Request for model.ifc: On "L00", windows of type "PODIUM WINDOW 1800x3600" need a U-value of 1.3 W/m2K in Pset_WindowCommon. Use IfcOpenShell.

First a look at what the model holds.

```python
import ifcopenshell
import ifcopenshell.util.element

model = ifcopenshell.open("model.ifc")
print(model.schema)
storey = next(s for s in model.by_type("IfcBuildingStorey") if s.Name == "L00")
windows = [e for e in ifcopenshell.util.element.get_decomposition(storey) if e.is_a("IfcWindow")]
seen = {}
for e in windows:
    element_type = ifcopenshell.util.element.get_type(e)
    key = (element_type.Name if element_type != e and element_type else None, ifcopenshell.util.element.get_pset(e, "Pset_WindowCommon", "ThermalTransmittance"))
    seen[key] = seen.get(key, 0) + 1
for (name, value), count in sorted(seen.items(), key=str):
    print(count, "x", name, "|", value)
```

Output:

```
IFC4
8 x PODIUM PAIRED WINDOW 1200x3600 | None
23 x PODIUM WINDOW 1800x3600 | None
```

```python
import ifcopenshell
import ifcopenshell.api.pset
import ifcopenshell.util.element

model = ifcopenshell.open("model.ifc")

storey = next(s for s in model.by_type("IfcBuildingStorey") if s.Name == "L00")
windows = [e for e in ifcopenshell.util.element.get_decomposition(storey) if e.is_a("IfcWindow")]

count = 0
for e in windows:
    element_type = ifcopenshell.util.element.get_type(e)
    if element_type in (None, e) or element_type.Name != "PODIUM WINDOW 1800x3600":
        continue
    # add_pset returns the element's existing set when there is one.
    pset = ifcopenshell.api.pset.add_pset(model, product=e, name="Pset_WindowCommon")
    ifcopenshell.api.pset.edit_pset(model, pset=pset, properties={"ThermalTransmittance": 1.3})
    count += 1

print(count, "windows updated")

model.write("model_edited.ifc")
```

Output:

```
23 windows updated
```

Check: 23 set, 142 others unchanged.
